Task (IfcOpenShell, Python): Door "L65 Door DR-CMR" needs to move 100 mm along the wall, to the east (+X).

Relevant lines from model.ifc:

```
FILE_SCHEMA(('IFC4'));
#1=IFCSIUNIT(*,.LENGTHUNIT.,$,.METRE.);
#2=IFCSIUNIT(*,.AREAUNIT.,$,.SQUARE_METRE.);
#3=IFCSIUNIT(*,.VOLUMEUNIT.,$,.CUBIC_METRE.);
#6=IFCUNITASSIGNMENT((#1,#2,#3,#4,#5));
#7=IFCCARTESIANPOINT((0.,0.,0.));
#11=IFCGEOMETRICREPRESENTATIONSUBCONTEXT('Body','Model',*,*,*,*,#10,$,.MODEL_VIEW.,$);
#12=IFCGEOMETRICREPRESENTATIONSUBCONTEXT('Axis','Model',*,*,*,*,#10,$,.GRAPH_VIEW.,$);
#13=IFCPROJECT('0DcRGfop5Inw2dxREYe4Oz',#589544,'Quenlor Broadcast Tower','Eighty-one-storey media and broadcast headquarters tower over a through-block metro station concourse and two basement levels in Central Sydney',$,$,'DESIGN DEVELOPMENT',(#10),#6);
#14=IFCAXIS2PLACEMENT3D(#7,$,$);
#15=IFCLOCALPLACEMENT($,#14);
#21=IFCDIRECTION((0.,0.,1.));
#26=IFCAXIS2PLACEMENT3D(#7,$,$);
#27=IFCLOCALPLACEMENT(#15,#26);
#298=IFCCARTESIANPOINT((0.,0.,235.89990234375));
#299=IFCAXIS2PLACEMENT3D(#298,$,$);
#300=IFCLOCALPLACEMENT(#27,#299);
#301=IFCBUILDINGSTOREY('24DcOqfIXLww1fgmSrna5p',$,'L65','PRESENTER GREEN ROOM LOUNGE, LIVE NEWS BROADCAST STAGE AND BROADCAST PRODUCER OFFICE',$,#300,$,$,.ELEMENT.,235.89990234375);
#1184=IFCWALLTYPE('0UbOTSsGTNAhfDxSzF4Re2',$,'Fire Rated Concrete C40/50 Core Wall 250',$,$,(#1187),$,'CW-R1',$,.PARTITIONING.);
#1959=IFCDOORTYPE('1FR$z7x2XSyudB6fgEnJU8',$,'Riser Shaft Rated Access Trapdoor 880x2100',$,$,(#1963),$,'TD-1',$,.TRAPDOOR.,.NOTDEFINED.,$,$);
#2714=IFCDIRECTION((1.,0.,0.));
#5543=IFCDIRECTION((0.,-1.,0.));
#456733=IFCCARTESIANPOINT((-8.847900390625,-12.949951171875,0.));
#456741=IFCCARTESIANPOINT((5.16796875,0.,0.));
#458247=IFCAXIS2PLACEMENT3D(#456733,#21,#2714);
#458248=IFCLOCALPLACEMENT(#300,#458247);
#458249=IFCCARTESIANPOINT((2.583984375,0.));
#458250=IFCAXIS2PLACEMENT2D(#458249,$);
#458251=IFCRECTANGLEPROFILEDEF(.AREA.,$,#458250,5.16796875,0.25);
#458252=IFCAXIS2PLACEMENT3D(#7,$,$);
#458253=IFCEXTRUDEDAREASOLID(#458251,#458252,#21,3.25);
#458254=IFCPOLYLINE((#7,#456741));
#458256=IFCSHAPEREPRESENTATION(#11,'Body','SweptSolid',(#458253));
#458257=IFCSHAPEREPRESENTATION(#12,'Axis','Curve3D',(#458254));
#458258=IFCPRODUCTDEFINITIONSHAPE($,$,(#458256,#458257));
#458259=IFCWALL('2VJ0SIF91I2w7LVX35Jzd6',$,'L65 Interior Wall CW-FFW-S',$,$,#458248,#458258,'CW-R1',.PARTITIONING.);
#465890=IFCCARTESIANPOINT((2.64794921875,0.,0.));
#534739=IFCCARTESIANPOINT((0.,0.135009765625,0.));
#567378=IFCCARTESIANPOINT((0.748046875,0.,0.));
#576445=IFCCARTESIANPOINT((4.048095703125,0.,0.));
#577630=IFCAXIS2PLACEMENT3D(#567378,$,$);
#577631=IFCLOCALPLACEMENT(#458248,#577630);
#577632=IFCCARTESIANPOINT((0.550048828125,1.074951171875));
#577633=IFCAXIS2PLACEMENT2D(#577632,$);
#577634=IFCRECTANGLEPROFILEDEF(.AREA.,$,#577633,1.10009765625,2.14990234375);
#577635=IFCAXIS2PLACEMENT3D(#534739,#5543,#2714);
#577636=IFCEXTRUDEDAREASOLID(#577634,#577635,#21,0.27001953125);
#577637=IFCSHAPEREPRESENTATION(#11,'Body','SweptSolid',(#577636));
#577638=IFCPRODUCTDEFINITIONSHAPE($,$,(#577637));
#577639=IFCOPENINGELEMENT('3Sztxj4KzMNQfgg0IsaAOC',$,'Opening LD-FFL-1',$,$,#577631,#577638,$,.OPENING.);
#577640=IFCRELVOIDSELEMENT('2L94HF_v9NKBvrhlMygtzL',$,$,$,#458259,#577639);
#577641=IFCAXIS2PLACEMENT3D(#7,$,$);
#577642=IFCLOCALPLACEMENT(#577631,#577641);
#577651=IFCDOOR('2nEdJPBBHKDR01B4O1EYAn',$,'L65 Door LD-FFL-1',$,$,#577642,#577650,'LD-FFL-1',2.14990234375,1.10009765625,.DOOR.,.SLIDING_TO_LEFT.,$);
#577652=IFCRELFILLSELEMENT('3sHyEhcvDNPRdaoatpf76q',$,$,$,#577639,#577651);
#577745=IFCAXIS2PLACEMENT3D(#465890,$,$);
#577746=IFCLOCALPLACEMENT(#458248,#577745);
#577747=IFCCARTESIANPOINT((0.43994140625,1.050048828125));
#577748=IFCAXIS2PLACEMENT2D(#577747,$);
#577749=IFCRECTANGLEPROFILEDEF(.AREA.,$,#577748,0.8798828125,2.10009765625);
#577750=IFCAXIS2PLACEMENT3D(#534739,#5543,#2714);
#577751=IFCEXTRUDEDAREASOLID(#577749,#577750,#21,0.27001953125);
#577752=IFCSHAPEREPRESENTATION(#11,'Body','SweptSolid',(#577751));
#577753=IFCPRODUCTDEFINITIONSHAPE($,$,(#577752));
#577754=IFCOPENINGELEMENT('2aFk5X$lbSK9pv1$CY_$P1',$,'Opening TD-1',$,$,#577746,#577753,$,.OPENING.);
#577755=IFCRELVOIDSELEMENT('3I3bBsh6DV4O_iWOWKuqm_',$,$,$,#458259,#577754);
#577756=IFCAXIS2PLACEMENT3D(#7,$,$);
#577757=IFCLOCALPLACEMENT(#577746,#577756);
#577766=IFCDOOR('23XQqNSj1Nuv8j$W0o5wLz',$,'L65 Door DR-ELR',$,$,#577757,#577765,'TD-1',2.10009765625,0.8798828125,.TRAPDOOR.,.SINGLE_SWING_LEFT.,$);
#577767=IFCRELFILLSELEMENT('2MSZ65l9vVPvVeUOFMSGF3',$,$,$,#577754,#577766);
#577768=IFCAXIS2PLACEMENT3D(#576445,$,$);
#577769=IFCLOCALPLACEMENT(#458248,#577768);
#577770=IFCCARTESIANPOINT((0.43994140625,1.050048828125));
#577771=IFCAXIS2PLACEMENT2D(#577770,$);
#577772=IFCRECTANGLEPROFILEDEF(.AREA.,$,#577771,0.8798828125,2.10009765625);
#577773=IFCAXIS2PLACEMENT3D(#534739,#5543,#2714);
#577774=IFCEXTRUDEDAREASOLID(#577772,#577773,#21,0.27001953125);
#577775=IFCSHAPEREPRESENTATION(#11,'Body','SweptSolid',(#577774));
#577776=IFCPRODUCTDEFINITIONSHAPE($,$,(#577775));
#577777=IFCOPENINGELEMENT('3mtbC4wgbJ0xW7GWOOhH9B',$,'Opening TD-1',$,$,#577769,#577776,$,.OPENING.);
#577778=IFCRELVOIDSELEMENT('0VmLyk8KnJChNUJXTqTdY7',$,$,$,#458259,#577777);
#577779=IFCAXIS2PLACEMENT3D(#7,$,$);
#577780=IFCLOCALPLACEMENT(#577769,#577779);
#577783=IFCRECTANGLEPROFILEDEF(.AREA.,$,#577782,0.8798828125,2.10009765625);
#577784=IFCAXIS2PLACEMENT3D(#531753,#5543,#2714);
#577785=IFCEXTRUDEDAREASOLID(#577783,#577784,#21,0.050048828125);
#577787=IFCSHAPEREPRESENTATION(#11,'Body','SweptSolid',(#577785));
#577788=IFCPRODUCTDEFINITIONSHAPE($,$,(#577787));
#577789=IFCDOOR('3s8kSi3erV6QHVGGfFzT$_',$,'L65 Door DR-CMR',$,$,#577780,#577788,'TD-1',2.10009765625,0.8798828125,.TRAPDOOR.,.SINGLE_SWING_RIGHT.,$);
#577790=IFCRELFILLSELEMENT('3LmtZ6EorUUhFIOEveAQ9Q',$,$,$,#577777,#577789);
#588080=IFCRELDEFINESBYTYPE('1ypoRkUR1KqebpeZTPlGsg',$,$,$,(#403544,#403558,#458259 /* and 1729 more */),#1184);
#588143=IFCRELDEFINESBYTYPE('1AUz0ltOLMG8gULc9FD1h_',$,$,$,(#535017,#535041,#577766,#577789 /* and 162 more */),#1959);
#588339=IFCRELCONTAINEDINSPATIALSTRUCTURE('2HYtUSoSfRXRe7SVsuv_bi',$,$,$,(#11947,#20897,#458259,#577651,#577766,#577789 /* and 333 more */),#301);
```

```python
import ifcopenshell
import ifcopenshell.api.geometry
import ifcopenshell.util.placement
import ifcopenshell.util.unit

model = ifcopenshell.open("model.ifc")
unit_scale = ifcopenshell.util.unit.calculate_unit_scale(model)

door = model.by_guid("3s8kSi3erV6QHVGGfFzT$_")
opening = door.FillsVoids[0].RelatingOpeningElement
wall = opening.VoidsElements[0].RelatingBuildingElement

wall_matrix = ifcopenshell.util.placement.get_local_placement(wall.ObjectPlacement)
shift = wall_matrix[:3, 0] * 0.1 / unit_scale
before = ifcopenshell.util.placement.get_local_placement(door.ObjectPlacement)[:3, 3].copy()

# The door is placed relative to its opening, so it follows when the opening moves.
matrix = ifcopenshell.util.placement.get_local_placement(opening.ObjectPlacement)
matrix[:3, 3] += shift
ifcopenshell.api.geometry.edit_object_placement(
    model, product=opening, matrix=matrix, is_si=False, should_transform_children=True
)

after = ifcopenshell.util.placement.get_local_placement(door.ObjectPlacement)[:3, 3]
print("door moved by", (after - before).round(3) + 0.0)

model.write("model_v2.ifc")
```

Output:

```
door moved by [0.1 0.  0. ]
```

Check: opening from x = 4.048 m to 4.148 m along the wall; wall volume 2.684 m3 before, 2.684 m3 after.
